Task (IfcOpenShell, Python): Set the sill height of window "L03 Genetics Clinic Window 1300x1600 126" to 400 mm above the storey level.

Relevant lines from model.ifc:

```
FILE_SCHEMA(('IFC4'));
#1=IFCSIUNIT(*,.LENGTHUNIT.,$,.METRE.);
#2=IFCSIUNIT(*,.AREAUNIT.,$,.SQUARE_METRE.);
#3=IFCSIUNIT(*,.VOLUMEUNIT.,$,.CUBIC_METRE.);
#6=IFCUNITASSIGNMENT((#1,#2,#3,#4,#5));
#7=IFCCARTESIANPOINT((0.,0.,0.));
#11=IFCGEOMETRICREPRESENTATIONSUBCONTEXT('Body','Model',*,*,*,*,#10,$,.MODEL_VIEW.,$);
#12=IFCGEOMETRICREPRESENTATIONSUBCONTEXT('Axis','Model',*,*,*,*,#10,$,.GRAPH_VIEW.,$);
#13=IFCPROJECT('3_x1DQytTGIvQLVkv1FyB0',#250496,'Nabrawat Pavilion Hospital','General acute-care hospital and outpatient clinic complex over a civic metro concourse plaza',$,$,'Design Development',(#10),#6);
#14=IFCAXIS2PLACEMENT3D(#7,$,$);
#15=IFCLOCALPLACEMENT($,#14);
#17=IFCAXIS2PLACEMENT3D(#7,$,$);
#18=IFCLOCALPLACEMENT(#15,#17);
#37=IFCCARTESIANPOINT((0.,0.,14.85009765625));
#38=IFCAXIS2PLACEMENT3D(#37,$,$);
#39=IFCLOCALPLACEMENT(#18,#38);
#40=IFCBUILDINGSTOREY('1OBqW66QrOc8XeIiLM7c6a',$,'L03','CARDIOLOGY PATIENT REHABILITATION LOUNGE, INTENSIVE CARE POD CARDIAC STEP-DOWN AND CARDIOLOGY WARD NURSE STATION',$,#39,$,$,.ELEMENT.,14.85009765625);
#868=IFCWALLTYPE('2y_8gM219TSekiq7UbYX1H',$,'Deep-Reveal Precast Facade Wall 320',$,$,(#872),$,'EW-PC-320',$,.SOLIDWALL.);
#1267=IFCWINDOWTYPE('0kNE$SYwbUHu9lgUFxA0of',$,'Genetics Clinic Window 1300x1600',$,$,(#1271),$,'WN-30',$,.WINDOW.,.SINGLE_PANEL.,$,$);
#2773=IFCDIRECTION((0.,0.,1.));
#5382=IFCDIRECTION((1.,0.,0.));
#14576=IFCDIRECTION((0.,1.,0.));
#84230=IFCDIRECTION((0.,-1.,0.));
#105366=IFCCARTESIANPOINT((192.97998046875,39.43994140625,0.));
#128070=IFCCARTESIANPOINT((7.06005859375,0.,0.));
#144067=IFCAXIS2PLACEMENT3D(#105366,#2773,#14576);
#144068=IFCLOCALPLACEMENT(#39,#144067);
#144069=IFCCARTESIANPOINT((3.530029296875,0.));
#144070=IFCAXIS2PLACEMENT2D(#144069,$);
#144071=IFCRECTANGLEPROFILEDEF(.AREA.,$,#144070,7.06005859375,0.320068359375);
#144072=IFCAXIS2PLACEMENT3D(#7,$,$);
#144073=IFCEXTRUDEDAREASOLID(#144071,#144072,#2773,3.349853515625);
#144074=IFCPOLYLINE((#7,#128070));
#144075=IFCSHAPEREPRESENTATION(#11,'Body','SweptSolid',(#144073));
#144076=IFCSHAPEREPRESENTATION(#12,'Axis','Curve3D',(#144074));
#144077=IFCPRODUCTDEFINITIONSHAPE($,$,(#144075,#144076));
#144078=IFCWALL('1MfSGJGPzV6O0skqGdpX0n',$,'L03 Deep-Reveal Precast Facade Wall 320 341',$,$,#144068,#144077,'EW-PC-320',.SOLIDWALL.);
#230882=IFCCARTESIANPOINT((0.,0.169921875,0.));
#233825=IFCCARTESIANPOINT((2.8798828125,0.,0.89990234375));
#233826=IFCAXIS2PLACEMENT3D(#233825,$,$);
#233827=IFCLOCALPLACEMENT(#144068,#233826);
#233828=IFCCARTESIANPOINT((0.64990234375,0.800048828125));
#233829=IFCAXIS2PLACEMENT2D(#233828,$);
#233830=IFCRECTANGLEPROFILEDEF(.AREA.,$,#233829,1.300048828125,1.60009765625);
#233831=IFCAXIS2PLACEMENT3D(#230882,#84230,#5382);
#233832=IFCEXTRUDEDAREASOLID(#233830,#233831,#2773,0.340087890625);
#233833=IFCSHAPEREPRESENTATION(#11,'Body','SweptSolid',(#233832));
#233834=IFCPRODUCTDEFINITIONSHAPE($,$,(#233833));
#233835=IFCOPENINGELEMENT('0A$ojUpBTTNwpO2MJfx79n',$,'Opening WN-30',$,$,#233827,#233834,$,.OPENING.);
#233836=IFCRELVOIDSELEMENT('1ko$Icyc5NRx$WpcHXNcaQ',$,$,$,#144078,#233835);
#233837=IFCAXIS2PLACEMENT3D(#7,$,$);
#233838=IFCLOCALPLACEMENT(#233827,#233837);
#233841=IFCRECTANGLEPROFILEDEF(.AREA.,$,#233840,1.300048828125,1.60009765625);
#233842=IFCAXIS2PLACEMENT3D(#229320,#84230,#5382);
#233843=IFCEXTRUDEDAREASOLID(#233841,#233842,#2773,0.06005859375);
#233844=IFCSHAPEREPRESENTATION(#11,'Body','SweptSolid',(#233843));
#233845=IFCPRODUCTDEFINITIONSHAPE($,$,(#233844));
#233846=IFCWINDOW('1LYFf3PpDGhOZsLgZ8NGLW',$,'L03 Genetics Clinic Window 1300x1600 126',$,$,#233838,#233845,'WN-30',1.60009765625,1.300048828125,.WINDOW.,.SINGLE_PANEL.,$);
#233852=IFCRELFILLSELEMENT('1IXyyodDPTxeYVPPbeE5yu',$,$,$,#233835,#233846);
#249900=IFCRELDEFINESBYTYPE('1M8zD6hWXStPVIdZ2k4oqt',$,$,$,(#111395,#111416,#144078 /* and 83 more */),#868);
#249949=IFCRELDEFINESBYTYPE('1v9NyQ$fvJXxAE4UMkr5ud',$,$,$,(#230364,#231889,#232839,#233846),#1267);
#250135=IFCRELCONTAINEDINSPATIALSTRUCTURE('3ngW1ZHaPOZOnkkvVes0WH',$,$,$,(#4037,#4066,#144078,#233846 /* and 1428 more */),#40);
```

```python
import numpy as np
import ifcopenshell
import ifcopenshell.api.geometry
import ifcopenshell.geom
import ifcopenshell.util.element
import ifcopenshell.util.placement
import ifcopenshell.util.shape
import ifcopenshell.util.unit

model = ifcopenshell.open("model.ifc")
unit_scale = ifcopenshell.util.unit.calculate_unit_scale(model)

window = model.by_id(233846)
opening = window.FillsVoids[0].RelatingOpeningElement
storey = ifcopenshell.util.element.get_container(window, ifc_class="IfcBuildingStorey")
level = ifcopenshell.util.placement.get_local_placement(storey.ObjectPlacement)[2, 3]

# The opening's origin need not be at the sill, so measure its lowest point.
shape = ifcopenshell.geom.create_shape(ifcopenshell.geom.settings(), opening)
bottom = ifcopenshell.util.shape.get_shape_bottom_elevation(shape, shape.geometry) / unit_scale
dz = level + 0.4 - bottom

shift = np.array([0.0, 0.0, dz])
# The window is placed relative to its opening, so it follows when the opening moves.
matrix = ifcopenshell.util.placement.get_local_placement(opening.ObjectPlacement)
matrix[:3, 3] += shift
ifcopenshell.api.geometry.edit_object_placement(
    model, product=opening, matrix=matrix, is_si=False, should_transform_children=True
)

print(f"moved by {dz * unit_scale:+.3f} m")

model.write("model_edited.ifc")
```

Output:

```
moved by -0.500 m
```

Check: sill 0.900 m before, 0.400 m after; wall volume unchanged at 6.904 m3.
